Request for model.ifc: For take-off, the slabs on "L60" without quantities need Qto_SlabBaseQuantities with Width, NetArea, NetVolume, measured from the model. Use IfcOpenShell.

First a look at what the model holds.

```python
import ifcopenshell
import ifcopenshell.util.element
import ifcopenshell.util.unit

model = ifcopenshell.open("model.ifc")
print(model.schema)
for unit_type in ("LENGTHUNIT", "AREAUNIT", "VOLUMEUNIT"):
    print(unit_type, ifcopenshell.util.unit.calculate_unit_scale(model, unit_type))
storey = next(s for s in model.by_type("IfcBuildingStorey") if s.Name == "L60")
slabs = [e for e in ifcopenshell.util.element.get_decomposition(storey) if e.is_a("IfcSlab")]
for e in sorted(slabs, key=lambda e: e.id()):
    print(e.id(), e.is_a(), e.Name, list(ifcopenshell.util.element.get_psets(e, qtos_only=True)), sep=" | ")
```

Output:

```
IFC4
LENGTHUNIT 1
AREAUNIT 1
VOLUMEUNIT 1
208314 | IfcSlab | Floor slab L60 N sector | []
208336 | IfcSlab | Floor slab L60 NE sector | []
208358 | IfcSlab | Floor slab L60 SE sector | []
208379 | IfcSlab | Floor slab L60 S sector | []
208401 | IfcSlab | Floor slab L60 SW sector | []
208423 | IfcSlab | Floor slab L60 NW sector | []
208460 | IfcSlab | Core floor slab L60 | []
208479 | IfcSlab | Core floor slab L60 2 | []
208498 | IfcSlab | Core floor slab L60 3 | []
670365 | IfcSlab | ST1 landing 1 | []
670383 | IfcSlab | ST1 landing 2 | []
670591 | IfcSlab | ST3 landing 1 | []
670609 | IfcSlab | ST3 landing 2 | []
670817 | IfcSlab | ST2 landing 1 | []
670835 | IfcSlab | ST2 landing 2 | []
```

```python
import ifcopenshell
import ifcopenshell.api.pset
import ifcopenshell.geom
import ifcopenshell.util.element
import ifcopenshell.util.shape
import ifcopenshell.util.unit

model = ifcopenshell.open("model.ifc")
unit_scale = ifcopenshell.util.unit.calculate_unit_scale(model)
area_scale = ifcopenshell.util.unit.calculate_unit_scale(model, "AREAUNIT")
volume_scale = ifcopenshell.util.unit.calculate_unit_scale(model, "VOLUMEUNIT")
settings = ifcopenshell.geom.settings()

storey = next(s for s in model.by_type("IfcBuildingStorey") if s.Name == "L60")
slabs = [e for e in ifcopenshell.util.element.get_decomposition(storey) if e.is_a("IfcSlab")]

for e in sorted(slabs, key=lambda e: e.id()):
    if ifcopenshell.util.element.get_psets(e, qtos_only=True, should_inherit=False):
        continue
    # Geometry comes back in metres, in the element's own axes.
    shape = ifcopenshell.geom.create_shape(settings, e)
    values = {
        "Width": ifcopenshell.util.shape.get_z(shape.geometry) / unit_scale,
        "NetArea": ifcopenshell.util.shape.get_footprint_area(shape.geometry) / area_scale,
        "NetVolume": ifcopenshell.util.shape.get_volume(shape.geometry) / volume_scale,
    }
    qto = ifcopenshell.api.pset.add_qto(model, product=e, name="Qto_SlabBaseQuantities")
    ifcopenshell.api.pset.edit_qto(model, qto=qto, properties=values)
    print(e.id(), {k: round(v, 3) for k, v in values.items()})

model.write("model_v2.ifc")
```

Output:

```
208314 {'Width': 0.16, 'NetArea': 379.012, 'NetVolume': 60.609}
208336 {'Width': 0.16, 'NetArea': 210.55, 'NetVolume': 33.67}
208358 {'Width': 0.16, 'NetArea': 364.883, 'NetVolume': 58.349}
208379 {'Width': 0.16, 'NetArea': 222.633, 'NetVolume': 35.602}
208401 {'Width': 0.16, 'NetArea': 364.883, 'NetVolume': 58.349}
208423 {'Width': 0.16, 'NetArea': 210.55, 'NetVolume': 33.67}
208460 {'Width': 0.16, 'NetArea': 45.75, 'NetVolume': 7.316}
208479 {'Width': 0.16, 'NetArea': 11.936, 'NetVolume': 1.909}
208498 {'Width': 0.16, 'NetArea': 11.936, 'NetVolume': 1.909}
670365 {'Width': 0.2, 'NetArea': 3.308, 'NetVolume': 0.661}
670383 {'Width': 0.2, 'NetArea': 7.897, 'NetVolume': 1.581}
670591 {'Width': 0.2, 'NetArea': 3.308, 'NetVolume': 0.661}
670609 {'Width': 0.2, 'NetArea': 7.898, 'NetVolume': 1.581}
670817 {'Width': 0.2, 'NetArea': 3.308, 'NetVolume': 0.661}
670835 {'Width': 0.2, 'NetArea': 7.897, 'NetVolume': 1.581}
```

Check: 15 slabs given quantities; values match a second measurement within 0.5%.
